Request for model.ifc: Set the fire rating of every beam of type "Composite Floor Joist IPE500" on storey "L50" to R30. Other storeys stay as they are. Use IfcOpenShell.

First a look at what the model holds.

```python
import ifcopenshell
import ifcopenshell.util.element

model = ifcopenshell.open("model.ifc")
print(model.schema)
storey = next(s for s in model.by_type("IfcBuildingStorey") if s.Name == "L50")
beams = [e for e in ifcopenshell.util.element.get_decomposition(storey) if e.is_a("IfcBeam")]
seen = {}
for e in beams:
    element_type = ifcopenshell.util.element.get_type(e)
    key = (element_type.Name if element_type != e and element_type else None, ifcopenshell.util.element.get_pset(e, "Pset_BeamCommon", "FireRating"))
    seen[key] = seen.get(key, 0) + 1
for (name, value), count in sorted(seen.items(), key=str):
    print(count, "x", name, "|", value)
```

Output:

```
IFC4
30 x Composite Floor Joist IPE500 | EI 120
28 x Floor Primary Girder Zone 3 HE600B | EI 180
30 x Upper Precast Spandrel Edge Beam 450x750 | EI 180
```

```python
import ifcopenshell
import ifcopenshell.api.pset
import ifcopenshell.util.element

model = ifcopenshell.open("model.ifc")

storey = next(s for s in model.by_type("IfcBuildingStorey") if s.Name == "L50")
beams = [e for e in ifcopenshell.util.element.get_decomposition(storey) if e.is_a("IfcBeam")]

count = 0
for e in beams:
    element_type = ifcopenshell.util.element.get_type(e)
    if element_type in (None, e) or element_type.Name != "Composite Floor Joist IPE500":
        continue
    # add_pset returns the element's existing set when there is one.
    pset = ifcopenshell.api.pset.add_pset(model, product=e, name="Pset_BeamCommon")
    ifcopenshell.api.pset.edit_pset(model, pset=pset, properties={"FireRating": "R30"})
    count += 1

print(count, "beams updated")

model.write("model-out.ifc")
```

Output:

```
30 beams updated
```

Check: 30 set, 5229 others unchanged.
